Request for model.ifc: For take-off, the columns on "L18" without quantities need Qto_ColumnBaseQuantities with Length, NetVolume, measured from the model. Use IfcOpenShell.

First a look at what the model holds.

```python
import ifcopenshell
import ifcopenshell.util.element
import ifcopenshell.util.unit

model = ifcopenshell.open("model.ifc")
print(model.schema)
for unit_type in ("LENGTHUNIT", "AREAUNIT", "VOLUMEUNIT"):
    print(unit_type, ifcopenshell.util.unit.calculate_unit_scale(model, unit_type))
storey = next(s for s in model.by_type("IfcBuildingStorey") if s.Name == "L18")
columns = [e for e in ifcopenshell.util.element.get_decomposition(storey) if e.is_a("IfcColumn")]
for e in sorted(columns, key=lambda e: e.id()):
    print(e.id(), e.is_a(), e.Name, list(ifcopenshell.util.element.get_psets(e, qtos_only=True)), sep=" | ")
```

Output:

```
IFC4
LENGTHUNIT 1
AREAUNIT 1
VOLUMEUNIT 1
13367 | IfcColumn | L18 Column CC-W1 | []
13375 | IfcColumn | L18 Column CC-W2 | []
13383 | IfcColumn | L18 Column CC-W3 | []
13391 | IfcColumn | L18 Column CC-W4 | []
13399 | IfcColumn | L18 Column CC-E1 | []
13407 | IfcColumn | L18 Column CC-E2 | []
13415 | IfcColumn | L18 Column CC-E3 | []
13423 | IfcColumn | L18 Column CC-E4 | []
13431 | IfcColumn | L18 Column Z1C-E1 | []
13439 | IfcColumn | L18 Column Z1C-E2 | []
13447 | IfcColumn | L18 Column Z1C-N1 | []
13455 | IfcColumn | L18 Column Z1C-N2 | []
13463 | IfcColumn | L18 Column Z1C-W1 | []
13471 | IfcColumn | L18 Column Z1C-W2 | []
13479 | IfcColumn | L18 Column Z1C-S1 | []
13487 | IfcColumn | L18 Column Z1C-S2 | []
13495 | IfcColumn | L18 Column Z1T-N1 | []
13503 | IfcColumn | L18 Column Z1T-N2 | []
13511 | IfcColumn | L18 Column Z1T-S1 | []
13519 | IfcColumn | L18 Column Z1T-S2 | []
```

```python
import ifcopenshell
import ifcopenshell.api.pset
import ifcopenshell.geom
import ifcopenshell.util.element
import ifcopenshell.util.shape
import ifcopenshell.util.unit

model = ifcopenshell.open("model.ifc")
unit_scale = ifcopenshell.util.unit.calculate_unit_scale(model)
volume_scale = ifcopenshell.util.unit.calculate_unit_scale(model, "VOLUMEUNIT")
settings = ifcopenshell.geom.settings()

storey = next(s for s in model.by_type("IfcBuildingStorey") if s.Name == "L18")
columns = [e for e in ifcopenshell.util.element.get_decomposition(storey) if e.is_a("IfcColumn")]

for e in sorted(columns, key=lambda e: e.id()):
    if ifcopenshell.util.element.get_psets(e, qtos_only=True, should_inherit=False):
        continue
    # Geometry comes back in metres, in the element's own axes.
    shape = ifcopenshell.geom.create_shape(settings, e)
    values = {
        "Length": ifcopenshell.util.shape.get_z(shape.geometry) / unit_scale,
        "NetVolume": ifcopenshell.util.shape.get_volume(shape.geometry) / volume_scale,
    }
    qto = ifcopenshell.api.pset.add_qto(model, product=e, name="Qto_ColumnBaseQuantities")
    ifcopenshell.api.pset.edit_qto(model, qto=qto, properties=values)
    print(e.id(), {k: round(v, 3) for k, v in values.items()})

model.write("model_updated.ifc")
```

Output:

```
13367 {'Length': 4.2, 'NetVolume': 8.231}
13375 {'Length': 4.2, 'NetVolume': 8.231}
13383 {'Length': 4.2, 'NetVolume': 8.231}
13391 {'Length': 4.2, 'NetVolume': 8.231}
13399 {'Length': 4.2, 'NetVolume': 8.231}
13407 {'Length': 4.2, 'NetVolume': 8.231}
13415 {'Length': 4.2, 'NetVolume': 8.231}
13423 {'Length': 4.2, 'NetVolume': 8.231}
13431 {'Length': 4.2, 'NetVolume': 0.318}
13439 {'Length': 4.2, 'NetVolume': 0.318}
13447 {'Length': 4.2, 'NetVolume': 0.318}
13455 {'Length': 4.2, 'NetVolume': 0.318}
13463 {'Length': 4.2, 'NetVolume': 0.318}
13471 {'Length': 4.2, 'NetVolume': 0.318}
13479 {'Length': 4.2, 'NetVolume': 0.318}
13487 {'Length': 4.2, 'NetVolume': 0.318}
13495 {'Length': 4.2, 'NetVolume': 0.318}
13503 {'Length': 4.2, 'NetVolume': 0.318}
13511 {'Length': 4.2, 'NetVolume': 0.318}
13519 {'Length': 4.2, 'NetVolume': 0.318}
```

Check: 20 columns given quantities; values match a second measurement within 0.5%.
